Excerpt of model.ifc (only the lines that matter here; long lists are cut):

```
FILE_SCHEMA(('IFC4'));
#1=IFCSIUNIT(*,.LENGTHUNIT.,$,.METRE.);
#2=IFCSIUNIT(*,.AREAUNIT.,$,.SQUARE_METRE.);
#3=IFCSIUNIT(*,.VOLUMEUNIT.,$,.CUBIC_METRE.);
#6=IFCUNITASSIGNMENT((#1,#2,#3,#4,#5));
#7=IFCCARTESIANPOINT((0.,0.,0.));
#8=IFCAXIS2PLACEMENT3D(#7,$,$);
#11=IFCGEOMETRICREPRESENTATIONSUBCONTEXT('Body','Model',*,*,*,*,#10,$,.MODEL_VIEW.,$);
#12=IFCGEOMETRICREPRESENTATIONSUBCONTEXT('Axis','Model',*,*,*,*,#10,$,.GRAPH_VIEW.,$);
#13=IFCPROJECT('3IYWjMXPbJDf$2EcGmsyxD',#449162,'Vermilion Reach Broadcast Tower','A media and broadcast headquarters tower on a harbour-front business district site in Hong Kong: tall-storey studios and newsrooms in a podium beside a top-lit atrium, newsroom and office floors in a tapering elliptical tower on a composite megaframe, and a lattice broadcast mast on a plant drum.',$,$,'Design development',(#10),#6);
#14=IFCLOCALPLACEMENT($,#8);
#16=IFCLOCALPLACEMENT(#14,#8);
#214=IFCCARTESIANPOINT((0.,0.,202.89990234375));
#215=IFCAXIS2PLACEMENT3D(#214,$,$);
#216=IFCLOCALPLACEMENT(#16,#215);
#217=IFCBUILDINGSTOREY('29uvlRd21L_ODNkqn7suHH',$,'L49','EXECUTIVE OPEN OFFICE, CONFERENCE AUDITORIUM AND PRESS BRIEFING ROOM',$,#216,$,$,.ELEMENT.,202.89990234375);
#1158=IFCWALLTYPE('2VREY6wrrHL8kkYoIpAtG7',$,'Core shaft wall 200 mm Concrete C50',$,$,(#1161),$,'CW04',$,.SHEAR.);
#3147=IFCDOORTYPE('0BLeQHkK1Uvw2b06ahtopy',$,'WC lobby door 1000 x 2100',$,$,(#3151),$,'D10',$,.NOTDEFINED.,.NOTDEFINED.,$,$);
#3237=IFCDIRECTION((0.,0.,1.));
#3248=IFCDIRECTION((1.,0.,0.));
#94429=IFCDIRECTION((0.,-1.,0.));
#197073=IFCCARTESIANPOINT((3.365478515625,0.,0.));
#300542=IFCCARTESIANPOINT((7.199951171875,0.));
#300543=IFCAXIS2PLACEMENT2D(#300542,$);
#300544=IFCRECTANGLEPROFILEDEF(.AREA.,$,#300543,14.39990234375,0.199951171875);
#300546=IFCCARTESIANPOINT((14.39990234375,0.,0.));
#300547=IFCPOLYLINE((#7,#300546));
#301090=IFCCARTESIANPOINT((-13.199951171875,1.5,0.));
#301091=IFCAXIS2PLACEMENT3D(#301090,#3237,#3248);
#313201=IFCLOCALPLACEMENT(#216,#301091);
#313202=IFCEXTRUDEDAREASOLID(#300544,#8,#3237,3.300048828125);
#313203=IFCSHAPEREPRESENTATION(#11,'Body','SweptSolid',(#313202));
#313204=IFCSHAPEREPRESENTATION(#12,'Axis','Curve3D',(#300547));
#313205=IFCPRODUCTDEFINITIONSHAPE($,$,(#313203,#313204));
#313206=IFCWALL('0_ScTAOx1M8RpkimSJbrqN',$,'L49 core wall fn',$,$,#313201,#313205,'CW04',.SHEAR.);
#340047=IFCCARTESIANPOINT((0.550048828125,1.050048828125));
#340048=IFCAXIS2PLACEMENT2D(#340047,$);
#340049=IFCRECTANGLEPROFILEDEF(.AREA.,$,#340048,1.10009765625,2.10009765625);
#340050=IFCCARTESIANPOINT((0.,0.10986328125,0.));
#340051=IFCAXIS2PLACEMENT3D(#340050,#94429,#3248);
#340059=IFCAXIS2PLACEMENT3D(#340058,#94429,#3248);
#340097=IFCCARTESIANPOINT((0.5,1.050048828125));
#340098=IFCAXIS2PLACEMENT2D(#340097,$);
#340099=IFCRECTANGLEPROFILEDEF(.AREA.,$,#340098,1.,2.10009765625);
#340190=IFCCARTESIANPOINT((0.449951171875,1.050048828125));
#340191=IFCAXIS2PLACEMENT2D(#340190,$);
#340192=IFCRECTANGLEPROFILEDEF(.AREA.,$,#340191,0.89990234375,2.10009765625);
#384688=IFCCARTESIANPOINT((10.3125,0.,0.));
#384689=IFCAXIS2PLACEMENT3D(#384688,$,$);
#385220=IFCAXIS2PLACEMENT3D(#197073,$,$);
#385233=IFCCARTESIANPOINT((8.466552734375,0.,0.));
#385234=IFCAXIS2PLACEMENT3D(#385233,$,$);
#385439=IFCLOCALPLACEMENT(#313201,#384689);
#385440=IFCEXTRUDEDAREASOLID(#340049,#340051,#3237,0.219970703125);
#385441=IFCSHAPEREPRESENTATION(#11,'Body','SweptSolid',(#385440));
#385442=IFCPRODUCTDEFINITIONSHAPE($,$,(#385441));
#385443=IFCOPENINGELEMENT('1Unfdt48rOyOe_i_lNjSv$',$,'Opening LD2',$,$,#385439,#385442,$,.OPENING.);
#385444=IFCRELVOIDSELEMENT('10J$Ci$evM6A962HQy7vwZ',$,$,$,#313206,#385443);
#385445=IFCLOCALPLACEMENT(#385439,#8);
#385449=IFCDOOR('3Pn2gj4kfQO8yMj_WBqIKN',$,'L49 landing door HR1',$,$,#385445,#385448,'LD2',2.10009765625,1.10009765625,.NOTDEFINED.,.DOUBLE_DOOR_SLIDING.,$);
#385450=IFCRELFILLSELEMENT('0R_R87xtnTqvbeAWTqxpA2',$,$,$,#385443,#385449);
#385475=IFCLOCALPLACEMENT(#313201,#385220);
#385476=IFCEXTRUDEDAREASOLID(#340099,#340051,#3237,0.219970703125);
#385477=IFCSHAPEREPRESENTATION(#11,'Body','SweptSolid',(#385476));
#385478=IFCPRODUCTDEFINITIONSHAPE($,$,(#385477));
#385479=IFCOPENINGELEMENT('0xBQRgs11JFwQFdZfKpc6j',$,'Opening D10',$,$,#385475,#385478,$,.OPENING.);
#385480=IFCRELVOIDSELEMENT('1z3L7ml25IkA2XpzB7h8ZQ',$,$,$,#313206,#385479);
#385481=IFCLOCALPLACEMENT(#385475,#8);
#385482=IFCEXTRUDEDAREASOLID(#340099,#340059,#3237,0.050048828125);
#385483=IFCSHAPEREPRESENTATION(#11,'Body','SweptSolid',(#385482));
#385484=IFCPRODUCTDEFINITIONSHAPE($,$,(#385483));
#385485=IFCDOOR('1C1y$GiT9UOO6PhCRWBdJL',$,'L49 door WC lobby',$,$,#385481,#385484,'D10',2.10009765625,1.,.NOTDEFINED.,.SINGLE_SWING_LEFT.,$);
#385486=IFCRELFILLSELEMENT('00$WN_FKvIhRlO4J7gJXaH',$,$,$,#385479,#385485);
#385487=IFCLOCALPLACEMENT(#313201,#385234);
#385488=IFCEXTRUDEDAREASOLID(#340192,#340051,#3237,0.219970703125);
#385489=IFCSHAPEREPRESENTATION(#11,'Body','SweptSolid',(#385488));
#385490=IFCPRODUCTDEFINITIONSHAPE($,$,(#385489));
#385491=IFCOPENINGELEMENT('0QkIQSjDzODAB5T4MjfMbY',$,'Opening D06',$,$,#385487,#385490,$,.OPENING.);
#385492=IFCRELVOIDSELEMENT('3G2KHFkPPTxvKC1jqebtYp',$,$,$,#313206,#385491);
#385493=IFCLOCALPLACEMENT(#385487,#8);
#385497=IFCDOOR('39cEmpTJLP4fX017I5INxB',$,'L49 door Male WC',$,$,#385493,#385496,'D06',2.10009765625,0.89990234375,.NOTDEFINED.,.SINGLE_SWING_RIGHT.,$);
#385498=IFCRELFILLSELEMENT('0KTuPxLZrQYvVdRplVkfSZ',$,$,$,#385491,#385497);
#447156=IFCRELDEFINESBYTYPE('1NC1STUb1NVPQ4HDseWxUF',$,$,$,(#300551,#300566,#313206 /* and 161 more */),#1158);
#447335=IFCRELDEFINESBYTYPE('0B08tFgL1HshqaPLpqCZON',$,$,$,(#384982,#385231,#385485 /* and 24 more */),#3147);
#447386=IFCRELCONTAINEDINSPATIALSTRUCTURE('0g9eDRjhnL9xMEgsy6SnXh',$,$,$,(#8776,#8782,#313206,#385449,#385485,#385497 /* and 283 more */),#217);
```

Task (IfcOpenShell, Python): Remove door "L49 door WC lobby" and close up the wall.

```python
import ifcopenshell
import ifcopenshell.api.feature
import ifcopenshell.api.root
import ifcopenshell.geom
import ifcopenshell.util.shape

model = ifcopenshell.open("model.ifc")
settings = ifcopenshell.geom.settings()


def volume(element):
    """Net volume in cubic metres, openings subtracted."""
    shape = ifcopenshell.geom.create_shape(settings, element)
    return ifcopenshell.util.shape.get_volume(shape.geometry)


door = model.by_guid("1C1y$GiT9UOO6PhCRWBdJL")
opening = door.FillsVoids[0].RelatingOpeningElement
wall = opening.VoidsElements[0].RelatingBuildingElement
before = volume(wall)

ifcopenshell.api.root.remove_product(model, product=door)
ifcopenshell.api.feature.remove_feature(model, feature=opening)

after = volume(wall)

print(f"wall volume {before:.3f} -> {after:.3f} m3")

model.write("model_v2.ifc")
```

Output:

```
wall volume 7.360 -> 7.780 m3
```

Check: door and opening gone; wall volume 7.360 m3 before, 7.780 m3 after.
